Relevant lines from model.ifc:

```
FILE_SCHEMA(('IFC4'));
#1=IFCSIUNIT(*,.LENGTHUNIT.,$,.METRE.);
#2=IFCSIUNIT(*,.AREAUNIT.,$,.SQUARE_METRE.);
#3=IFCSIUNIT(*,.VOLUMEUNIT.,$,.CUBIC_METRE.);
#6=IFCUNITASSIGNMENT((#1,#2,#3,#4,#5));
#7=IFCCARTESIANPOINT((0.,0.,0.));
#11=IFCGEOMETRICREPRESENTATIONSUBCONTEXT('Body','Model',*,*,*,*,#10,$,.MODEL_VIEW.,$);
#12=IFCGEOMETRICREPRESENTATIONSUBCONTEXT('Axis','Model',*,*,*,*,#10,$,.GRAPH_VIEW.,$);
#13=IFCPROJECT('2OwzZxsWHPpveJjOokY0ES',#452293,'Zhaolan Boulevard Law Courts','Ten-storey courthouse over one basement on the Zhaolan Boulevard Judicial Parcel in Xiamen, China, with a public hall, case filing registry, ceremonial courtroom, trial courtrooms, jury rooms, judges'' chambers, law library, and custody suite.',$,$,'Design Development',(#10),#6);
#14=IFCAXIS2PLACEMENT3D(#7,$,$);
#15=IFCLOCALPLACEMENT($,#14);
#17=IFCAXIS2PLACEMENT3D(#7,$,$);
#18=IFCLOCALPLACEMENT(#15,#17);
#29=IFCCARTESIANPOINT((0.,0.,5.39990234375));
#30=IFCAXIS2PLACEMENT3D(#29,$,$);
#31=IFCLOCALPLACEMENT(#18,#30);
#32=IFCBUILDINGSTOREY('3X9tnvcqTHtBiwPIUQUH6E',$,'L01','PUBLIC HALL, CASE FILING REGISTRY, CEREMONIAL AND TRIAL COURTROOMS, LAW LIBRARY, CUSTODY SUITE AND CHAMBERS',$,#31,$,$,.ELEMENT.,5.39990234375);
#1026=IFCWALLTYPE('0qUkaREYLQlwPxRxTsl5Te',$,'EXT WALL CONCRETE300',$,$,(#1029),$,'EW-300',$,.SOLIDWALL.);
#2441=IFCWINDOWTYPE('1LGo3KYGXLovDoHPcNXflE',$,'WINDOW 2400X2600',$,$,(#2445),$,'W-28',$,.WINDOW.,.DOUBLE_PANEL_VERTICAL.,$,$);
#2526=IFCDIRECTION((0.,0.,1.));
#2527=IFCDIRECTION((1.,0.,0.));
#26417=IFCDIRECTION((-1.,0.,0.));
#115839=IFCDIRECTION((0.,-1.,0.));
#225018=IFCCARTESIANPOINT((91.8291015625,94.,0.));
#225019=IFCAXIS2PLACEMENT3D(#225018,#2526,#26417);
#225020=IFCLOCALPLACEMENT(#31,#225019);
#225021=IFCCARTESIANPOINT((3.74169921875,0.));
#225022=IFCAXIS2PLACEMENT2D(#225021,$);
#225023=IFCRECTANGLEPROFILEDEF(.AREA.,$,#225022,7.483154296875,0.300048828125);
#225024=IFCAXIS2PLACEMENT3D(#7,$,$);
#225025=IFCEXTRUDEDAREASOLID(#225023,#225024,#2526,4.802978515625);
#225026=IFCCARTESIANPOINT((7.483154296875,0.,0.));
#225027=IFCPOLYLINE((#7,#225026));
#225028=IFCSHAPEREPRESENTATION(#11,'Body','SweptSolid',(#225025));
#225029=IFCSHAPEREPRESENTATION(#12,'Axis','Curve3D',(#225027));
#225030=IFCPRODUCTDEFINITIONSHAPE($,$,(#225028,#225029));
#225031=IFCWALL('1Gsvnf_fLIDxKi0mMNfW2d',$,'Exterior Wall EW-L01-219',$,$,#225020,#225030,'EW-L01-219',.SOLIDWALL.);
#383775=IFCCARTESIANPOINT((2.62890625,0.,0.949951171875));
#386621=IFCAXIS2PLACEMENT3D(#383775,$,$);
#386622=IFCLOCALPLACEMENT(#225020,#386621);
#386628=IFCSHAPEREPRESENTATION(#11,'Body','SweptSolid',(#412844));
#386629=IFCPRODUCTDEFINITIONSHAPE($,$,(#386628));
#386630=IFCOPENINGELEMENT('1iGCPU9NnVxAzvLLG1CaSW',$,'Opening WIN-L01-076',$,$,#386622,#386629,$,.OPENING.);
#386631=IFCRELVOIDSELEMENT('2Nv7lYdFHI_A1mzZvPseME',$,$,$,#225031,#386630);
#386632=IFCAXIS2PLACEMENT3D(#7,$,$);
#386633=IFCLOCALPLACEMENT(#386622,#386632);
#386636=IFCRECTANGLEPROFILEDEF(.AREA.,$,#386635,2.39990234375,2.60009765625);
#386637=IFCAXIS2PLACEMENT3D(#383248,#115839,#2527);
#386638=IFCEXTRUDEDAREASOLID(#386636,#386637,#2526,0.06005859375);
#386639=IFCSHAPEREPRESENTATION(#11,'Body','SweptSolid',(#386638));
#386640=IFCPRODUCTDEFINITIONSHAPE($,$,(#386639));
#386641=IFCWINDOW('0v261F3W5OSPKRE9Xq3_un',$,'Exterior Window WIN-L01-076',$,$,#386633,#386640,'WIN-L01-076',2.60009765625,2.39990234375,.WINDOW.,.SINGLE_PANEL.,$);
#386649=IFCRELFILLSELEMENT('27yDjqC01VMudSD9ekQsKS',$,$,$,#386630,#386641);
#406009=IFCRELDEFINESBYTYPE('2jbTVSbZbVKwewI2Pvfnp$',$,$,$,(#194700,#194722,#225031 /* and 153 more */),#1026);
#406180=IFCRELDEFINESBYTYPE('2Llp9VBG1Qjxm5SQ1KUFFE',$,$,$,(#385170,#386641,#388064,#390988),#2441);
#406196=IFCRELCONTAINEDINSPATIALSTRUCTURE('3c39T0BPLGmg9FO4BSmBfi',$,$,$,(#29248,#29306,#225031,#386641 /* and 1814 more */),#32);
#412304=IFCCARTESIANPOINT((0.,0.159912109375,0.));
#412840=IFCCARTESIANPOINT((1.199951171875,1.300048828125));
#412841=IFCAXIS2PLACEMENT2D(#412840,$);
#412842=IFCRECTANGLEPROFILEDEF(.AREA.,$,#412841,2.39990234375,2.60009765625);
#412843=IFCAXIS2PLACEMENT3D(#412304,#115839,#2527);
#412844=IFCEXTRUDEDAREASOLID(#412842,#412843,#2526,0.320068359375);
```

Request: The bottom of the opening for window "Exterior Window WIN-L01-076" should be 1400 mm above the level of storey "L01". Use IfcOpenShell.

```python
import numpy as np
import ifcopenshell
import ifcopenshell.api.geometry
import ifcopenshell.geom
import ifcopenshell.util.element
import ifcopenshell.util.placement
import ifcopenshell.util.shape
import ifcopenshell.util.unit

model = ifcopenshell.open("model.ifc")
unit_scale = ifcopenshell.util.unit.calculate_unit_scale(model)

window = model.by_id(386641)
opening = window.FillsVoids[0].RelatingOpeningElement
storey = ifcopenshell.util.element.get_container(window, ifc_class="IfcBuildingStorey")
level = ifcopenshell.util.placement.get_local_placement(storey.ObjectPlacement)[2, 3]

# The opening's origin need not be at the sill, so measure its lowest point.
shape = ifcopenshell.geom.create_shape(ifcopenshell.geom.settings(), opening)
bottom = ifcopenshell.util.shape.get_shape_bottom_elevation(shape, shape.geometry) / unit_scale
dz = level + 1.4 / unit_scale - bottom

shift = np.array([0.0, 0.0, dz])
# The window is placed relative to its opening, so it follows when the opening moves.
matrix = ifcopenshell.util.placement.get_local_placement(opening.ObjectPlacement)
matrix[:3, 3] += shift
ifcopenshell.api.geometry.edit_object_placement(
    model, product=opening, matrix=matrix, is_si=False, should_transform_children=True
)

print(f"moved by {dz * unit_scale:+.3f} m")

model.write("model-out.ifc")
```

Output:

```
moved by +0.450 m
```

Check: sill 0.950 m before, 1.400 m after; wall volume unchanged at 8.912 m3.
